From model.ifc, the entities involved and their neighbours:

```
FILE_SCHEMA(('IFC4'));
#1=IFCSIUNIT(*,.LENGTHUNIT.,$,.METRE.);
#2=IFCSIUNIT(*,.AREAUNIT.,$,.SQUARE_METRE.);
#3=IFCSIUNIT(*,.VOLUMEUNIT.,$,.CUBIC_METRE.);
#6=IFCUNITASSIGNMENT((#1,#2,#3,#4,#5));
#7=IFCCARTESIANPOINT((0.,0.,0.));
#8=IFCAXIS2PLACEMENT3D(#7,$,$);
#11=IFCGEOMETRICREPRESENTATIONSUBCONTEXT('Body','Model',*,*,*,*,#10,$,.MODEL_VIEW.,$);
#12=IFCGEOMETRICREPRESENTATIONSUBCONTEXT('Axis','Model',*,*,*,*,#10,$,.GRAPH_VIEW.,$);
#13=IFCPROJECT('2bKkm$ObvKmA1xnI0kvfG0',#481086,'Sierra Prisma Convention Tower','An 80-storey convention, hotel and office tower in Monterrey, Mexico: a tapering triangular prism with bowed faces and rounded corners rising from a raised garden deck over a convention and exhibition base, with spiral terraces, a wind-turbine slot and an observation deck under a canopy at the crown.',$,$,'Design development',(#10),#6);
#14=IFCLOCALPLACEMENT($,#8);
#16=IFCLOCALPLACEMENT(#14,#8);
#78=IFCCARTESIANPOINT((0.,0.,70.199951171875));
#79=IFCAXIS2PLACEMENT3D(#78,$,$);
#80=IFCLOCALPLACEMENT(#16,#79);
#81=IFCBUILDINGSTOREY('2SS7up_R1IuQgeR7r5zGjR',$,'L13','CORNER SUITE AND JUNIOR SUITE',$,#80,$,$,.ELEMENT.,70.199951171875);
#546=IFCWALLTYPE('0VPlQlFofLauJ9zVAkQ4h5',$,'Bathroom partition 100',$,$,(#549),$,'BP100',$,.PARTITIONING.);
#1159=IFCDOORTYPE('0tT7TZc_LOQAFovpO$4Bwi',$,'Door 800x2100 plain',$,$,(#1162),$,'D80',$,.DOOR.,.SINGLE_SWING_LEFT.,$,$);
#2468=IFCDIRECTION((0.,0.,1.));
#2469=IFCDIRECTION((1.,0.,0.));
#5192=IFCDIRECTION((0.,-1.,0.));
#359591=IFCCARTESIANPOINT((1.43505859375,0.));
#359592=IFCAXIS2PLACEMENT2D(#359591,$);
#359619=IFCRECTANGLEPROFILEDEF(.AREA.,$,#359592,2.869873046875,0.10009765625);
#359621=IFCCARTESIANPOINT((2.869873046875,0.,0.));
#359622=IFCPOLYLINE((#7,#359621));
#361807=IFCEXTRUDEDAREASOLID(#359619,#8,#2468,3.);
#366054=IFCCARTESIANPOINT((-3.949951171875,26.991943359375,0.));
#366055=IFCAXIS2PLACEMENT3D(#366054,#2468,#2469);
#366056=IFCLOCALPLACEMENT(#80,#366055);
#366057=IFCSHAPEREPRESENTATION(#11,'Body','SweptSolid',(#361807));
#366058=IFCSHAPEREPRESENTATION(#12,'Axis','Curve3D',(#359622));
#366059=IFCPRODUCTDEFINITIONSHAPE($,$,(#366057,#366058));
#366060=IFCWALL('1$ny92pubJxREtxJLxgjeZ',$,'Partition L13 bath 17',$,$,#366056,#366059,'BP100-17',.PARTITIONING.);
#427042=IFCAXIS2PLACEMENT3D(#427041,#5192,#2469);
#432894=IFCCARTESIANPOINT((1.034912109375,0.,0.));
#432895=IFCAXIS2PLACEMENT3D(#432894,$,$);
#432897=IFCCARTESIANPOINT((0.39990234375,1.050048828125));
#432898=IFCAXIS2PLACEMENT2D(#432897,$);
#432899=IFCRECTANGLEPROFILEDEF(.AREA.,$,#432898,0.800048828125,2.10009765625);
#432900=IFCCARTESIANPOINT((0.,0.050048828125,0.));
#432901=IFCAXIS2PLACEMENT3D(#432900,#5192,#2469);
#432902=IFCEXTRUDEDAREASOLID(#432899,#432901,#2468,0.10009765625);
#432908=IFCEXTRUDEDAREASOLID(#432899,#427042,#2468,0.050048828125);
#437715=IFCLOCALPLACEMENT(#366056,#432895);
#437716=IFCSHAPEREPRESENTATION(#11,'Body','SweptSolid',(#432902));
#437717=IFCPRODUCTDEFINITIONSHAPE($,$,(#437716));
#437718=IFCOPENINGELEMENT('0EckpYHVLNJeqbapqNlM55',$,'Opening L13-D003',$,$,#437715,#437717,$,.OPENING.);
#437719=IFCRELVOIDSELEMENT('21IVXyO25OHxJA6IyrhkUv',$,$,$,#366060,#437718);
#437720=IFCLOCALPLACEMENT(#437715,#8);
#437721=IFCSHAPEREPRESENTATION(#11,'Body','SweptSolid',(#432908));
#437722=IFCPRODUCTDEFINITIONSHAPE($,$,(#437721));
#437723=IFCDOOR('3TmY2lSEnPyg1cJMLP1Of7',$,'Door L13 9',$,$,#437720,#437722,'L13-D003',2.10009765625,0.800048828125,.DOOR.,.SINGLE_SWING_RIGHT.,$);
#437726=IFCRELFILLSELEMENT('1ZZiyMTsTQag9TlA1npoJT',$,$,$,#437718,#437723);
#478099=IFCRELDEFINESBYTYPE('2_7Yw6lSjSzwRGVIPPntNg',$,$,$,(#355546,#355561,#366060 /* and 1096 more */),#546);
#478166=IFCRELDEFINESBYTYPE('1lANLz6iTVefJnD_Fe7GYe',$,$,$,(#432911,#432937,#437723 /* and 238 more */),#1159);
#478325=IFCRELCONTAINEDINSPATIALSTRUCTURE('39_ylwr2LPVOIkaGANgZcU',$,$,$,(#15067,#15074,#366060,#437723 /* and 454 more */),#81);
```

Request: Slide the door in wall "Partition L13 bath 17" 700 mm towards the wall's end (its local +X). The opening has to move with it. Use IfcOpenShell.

```python
import ifcopenshell
import ifcopenshell.api.geometry
import ifcopenshell.util.placement
import ifcopenshell.util.unit

model = ifcopenshell.open("model.ifc")
unit_scale = ifcopenshell.util.unit.calculate_unit_scale(model)

door = model.by_id(437723)
opening = door.FillsVoids[0].RelatingOpeningElement
wall = opening.VoidsElements[0].RelatingBuildingElement

wall_matrix = ifcopenshell.util.placement.get_local_placement(wall.ObjectPlacement)
shift = wall_matrix[:3, 0] * 0.7 / unit_scale
before = ifcopenshell.util.placement.get_local_placement(door.ObjectPlacement)[:3, 3].copy()

# The door is placed relative to its opening, so it follows when the opening moves.
matrix = ifcopenshell.util.placement.get_local_placement(opening.ObjectPlacement)
matrix[:3, 3] += shift
ifcopenshell.api.geometry.edit_object_placement(
    model, product=opening, matrix=matrix, is_si=False, should_transform_children=True
)

after = ifcopenshell.util.placement.get_local_placement(door.ObjectPlacement)[:3, 3]
print("door moved by", (after - before).round(3) + 0.0)

model.write("model-out.ifc")
```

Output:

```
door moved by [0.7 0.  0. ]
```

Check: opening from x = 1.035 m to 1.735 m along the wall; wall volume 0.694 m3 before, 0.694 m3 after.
